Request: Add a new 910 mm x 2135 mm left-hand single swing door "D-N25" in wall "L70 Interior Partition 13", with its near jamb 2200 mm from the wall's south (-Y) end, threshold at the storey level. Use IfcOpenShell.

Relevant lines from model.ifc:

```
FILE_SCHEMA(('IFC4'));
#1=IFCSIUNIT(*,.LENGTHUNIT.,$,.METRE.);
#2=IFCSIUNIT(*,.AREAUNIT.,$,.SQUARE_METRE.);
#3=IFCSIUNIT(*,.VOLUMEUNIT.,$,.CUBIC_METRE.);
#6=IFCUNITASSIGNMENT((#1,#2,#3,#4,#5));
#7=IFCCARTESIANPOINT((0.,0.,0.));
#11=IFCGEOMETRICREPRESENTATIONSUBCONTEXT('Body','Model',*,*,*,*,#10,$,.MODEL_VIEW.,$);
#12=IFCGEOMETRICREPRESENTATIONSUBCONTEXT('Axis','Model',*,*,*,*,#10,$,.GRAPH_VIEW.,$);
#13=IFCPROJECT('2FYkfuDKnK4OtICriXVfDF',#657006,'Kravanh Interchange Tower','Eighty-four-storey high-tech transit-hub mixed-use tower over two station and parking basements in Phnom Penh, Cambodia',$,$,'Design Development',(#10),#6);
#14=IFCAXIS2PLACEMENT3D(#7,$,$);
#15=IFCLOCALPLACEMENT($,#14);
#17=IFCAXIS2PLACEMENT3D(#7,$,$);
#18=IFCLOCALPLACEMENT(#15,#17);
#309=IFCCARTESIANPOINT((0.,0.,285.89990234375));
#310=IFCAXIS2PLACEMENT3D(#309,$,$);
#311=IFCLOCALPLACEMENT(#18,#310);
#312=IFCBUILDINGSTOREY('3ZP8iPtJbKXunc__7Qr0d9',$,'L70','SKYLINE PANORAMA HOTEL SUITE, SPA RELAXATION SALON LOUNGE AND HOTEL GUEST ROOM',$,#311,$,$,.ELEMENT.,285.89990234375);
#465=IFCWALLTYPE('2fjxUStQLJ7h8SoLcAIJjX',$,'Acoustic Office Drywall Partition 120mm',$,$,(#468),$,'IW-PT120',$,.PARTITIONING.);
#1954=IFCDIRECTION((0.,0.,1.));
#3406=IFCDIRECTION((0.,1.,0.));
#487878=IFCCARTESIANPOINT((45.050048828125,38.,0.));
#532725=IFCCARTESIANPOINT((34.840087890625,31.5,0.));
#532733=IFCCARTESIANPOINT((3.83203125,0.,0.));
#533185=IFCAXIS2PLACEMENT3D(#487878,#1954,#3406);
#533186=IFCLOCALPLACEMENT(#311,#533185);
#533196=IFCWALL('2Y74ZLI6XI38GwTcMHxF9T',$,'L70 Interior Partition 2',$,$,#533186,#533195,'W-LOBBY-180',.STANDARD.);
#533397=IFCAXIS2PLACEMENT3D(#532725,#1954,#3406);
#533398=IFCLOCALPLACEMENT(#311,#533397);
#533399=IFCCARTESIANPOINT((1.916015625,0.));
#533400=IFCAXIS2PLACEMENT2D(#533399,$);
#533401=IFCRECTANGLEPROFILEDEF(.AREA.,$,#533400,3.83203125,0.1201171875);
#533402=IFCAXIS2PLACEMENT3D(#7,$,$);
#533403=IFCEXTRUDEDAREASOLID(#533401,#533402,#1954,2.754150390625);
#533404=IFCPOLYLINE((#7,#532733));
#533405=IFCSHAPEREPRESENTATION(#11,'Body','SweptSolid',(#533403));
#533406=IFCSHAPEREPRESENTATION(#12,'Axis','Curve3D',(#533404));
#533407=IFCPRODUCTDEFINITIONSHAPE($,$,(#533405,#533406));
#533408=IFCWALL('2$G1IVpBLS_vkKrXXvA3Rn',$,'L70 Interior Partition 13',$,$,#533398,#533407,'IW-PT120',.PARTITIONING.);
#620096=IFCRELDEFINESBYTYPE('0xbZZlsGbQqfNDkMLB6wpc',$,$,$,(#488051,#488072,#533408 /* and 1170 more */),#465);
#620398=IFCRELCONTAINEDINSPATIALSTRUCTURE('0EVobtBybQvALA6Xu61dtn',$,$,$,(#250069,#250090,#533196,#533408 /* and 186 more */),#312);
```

```python
import numpy as np
import ifcopenshell
import ifcopenshell.api.feature
import ifcopenshell.api.geometry
import ifcopenshell.api.root
import ifcopenshell.api.spatial
import ifcopenshell.geom
import ifcopenshell.util.element
import ifcopenshell.util.placement
import ifcopenshell.util.representation
import ifcopenshell.util.shape
import ifcopenshell.util.unit

model = ifcopenshell.open("model.ifc")
unit_scale = ifcopenshell.util.unit.calculate_unit_scale(model)
settings = ifcopenshell.geom.settings()


def volume(element):
    """Net volume in cubic metres, openings subtracted."""
    shape = ifcopenshell.geom.create_shape(settings, element)
    return ifcopenshell.util.shape.get_volume(shape.geometry)


wall = model.by_guid("2$G1IVpBLS_vkKrXXvA3Rn")
storey = ifcopenshell.util.element.get_container(wall, ifc_class="IfcBuildingStorey")
context = ifcopenshell.util.representation.get_context(model, "Model", "Body", "MODEL_VIEW")
before = volume(wall)

width, height, from_end, sill = 0.91, 2.135, 2.2, 0.0  # metres

# The wall runs along its own X axis, and the end named is its -X end.
wall_shape = ifcopenshell.geom.create_shape(settings, wall)
x, y, z = ifcopenshell.util.shape.get_vertices(wall_shape.geometry).T
start = x.min() + from_end
face, thickness = float(y.min()), float(y.max() - y.min())
wall_matrix = ifcopenshell.util.placement.get_local_placement(wall.ObjectPlacement)
level = ifcopenshell.util.placement.get_local_placement(storey.ObjectPlacement)[2, 3]


def in_wall(x, y):
    """Placement at x, y metres in the wall's axes, at sill height."""
    matrix = wall_matrix.copy()
    matrix[:, 3] = wall_matrix @ np.array([x / unit_scale, y / unit_scale, 0.0, 1.0])
    matrix[2, 3] = level + sill / unit_scale
    return matrix


# Opening: a box that overshoots both wall faces by 50 mm.
opening = ifcopenshell.api.root.create_entity(model, ifc_class="IfcOpeningElement", predefined_type="OPENING")
box = ifcopenshell.api.geometry.add_wall_representation(
    model, context=context, length=width, height=height, thickness=thickness + 0.1
)
ifcopenshell.api.geometry.assign_representation(model, product=opening, representation=box)
ifcopenshell.api.geometry.edit_object_placement(model, product=opening, matrix=in_wall(start, face - 0.05), is_si=False)
ifcopenshell.api.feature.add_feature(model, feature=opening, element=wall)

door = ifcopenshell.api.root.create_entity(model, ifc_class="IfcDoor", name="D-N25", predefined_type="DOOR")
door.OverallWidth, door.OverallHeight = width / unit_scale, height / unit_scale
door.OperationType = "SINGLE_SWING_LEFT"
body = ifcopenshell.api.geometry.add_door_representation(
    model,
    context=context,
    overall_width=door.OverallWidth,
    overall_height=door.OverallHeight,
    operation_type="SINGLE_SWING_LEFT",
    lining_properties={"LiningDepth": thickness / unit_scale, "ThresholdDepth": thickness / unit_scale},
)
ifcopenshell.api.geometry.assign_representation(model, product=door, representation=body)
ifcopenshell.api.spatial.assign_container(model, products=[door], relating_structure=storey)
ifcopenshell.api.feature.add_filling(model, opening=opening, element=door)

# The lining spans the wall, so the door starts at the wall face.
ifcopenshell.api.geometry.edit_object_placement(model, product=door, matrix=in_wall(start, face), is_si=False)

after = volume(wall)

print(f"wall volume {before:.3f} -> {after:.3f} m3")

model.write("model-out.ifc")
```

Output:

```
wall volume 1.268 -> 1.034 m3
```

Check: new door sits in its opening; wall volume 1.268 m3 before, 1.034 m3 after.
